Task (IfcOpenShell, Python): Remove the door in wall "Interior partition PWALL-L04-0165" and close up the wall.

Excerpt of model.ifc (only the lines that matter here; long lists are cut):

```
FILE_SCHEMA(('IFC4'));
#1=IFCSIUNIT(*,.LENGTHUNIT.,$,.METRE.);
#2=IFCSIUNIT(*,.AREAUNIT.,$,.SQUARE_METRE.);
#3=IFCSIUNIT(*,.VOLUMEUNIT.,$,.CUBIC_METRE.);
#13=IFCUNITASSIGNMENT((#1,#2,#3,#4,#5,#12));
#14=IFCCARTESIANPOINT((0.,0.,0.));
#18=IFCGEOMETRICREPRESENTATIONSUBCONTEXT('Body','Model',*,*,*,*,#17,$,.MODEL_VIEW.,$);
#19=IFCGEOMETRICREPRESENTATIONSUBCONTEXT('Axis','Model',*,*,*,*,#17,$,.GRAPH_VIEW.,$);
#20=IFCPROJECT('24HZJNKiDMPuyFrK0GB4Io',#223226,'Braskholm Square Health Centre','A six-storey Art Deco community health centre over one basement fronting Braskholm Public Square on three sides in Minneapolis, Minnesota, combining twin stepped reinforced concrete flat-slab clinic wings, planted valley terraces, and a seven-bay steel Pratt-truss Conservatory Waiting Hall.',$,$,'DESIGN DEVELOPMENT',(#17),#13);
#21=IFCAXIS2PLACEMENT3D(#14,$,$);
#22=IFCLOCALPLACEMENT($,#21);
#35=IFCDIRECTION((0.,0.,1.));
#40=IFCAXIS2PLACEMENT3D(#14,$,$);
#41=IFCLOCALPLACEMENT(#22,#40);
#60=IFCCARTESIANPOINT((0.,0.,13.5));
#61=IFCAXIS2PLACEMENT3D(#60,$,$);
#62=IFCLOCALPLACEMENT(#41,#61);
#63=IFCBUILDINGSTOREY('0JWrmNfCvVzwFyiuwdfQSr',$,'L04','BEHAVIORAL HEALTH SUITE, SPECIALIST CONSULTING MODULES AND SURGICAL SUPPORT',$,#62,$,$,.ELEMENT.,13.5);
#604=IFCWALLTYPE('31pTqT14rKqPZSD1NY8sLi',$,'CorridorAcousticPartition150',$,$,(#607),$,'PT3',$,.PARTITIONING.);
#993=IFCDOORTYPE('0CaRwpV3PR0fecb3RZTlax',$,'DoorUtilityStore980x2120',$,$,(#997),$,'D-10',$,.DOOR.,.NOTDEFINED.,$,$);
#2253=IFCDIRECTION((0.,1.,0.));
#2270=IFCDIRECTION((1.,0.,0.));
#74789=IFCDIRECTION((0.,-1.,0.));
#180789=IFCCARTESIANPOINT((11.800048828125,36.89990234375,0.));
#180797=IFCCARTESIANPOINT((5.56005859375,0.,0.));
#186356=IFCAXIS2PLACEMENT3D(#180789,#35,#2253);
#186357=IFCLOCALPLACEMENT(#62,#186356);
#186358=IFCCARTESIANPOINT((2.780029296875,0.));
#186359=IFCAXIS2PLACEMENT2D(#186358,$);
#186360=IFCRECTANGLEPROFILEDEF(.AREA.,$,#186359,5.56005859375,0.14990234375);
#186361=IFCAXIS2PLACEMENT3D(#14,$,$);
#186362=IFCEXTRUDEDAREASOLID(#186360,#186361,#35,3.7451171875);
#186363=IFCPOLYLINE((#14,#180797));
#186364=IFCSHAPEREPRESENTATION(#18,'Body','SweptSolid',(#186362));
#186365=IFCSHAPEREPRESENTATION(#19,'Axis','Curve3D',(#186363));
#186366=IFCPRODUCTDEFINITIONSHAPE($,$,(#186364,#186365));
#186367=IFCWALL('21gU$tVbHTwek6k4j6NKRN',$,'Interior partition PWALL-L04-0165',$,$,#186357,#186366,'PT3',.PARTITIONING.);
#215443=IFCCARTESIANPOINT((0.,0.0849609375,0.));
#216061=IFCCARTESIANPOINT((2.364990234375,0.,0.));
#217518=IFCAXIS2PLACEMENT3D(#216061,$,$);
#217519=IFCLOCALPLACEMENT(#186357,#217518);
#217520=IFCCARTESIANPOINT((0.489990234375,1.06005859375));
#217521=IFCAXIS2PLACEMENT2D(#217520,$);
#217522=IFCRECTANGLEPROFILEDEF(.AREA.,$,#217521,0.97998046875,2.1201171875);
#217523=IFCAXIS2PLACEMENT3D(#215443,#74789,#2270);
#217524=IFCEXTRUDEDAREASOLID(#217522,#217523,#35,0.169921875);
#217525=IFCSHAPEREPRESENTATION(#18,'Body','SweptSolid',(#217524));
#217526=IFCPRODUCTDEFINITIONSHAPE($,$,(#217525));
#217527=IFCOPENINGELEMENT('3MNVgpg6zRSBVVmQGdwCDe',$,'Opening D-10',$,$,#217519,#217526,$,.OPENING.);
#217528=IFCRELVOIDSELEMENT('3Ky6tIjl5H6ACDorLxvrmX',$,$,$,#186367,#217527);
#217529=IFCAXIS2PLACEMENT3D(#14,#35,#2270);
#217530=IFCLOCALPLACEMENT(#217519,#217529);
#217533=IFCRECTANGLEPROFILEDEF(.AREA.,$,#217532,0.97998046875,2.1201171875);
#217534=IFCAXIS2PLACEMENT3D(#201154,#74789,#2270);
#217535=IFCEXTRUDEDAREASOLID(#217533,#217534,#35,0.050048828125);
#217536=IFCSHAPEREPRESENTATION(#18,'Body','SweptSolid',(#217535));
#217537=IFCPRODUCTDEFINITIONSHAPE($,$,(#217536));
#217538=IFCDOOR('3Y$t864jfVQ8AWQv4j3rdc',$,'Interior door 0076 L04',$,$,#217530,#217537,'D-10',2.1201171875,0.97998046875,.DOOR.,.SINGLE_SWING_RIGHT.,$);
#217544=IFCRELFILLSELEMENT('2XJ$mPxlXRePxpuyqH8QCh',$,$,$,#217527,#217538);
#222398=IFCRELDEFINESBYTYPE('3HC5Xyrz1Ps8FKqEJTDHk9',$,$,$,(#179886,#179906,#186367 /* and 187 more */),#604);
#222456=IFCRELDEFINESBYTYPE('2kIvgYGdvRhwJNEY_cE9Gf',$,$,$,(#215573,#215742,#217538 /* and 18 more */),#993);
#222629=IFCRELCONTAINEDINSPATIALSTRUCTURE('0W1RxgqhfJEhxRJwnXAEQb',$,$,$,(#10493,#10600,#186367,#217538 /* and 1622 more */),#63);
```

```python
import ifcopenshell
import ifcopenshell.api.feature
import ifcopenshell.api.root
import ifcopenshell.geom
import ifcopenshell.util.shape

model = ifcopenshell.open("model.ifc")
settings = ifcopenshell.geom.settings()


def volume(element):
    """Net volume in cubic metres, openings subtracted."""
    shape = ifcopenshell.geom.create_shape(settings, element)
    return ifcopenshell.util.shape.get_volume(shape.geometry)


door = model.by_guid("3Y$t864jfVQ8AWQv4j3rdc")
opening = door.FillsVoids[0].RelatingOpeningElement
wall = opening.VoidsElements[0].RelatingBuildingElement
before = volume(wall)

ifcopenshell.api.root.remove_product(model, product=door)
ifcopenshell.api.feature.remove_feature(model, feature=opening)

after = volume(wall)

print(f"wall volume {before:.3f} -> {after:.3f} m3")

model.write("model_edited.ifc")
```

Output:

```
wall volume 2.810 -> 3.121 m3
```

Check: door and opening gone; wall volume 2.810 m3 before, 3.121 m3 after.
